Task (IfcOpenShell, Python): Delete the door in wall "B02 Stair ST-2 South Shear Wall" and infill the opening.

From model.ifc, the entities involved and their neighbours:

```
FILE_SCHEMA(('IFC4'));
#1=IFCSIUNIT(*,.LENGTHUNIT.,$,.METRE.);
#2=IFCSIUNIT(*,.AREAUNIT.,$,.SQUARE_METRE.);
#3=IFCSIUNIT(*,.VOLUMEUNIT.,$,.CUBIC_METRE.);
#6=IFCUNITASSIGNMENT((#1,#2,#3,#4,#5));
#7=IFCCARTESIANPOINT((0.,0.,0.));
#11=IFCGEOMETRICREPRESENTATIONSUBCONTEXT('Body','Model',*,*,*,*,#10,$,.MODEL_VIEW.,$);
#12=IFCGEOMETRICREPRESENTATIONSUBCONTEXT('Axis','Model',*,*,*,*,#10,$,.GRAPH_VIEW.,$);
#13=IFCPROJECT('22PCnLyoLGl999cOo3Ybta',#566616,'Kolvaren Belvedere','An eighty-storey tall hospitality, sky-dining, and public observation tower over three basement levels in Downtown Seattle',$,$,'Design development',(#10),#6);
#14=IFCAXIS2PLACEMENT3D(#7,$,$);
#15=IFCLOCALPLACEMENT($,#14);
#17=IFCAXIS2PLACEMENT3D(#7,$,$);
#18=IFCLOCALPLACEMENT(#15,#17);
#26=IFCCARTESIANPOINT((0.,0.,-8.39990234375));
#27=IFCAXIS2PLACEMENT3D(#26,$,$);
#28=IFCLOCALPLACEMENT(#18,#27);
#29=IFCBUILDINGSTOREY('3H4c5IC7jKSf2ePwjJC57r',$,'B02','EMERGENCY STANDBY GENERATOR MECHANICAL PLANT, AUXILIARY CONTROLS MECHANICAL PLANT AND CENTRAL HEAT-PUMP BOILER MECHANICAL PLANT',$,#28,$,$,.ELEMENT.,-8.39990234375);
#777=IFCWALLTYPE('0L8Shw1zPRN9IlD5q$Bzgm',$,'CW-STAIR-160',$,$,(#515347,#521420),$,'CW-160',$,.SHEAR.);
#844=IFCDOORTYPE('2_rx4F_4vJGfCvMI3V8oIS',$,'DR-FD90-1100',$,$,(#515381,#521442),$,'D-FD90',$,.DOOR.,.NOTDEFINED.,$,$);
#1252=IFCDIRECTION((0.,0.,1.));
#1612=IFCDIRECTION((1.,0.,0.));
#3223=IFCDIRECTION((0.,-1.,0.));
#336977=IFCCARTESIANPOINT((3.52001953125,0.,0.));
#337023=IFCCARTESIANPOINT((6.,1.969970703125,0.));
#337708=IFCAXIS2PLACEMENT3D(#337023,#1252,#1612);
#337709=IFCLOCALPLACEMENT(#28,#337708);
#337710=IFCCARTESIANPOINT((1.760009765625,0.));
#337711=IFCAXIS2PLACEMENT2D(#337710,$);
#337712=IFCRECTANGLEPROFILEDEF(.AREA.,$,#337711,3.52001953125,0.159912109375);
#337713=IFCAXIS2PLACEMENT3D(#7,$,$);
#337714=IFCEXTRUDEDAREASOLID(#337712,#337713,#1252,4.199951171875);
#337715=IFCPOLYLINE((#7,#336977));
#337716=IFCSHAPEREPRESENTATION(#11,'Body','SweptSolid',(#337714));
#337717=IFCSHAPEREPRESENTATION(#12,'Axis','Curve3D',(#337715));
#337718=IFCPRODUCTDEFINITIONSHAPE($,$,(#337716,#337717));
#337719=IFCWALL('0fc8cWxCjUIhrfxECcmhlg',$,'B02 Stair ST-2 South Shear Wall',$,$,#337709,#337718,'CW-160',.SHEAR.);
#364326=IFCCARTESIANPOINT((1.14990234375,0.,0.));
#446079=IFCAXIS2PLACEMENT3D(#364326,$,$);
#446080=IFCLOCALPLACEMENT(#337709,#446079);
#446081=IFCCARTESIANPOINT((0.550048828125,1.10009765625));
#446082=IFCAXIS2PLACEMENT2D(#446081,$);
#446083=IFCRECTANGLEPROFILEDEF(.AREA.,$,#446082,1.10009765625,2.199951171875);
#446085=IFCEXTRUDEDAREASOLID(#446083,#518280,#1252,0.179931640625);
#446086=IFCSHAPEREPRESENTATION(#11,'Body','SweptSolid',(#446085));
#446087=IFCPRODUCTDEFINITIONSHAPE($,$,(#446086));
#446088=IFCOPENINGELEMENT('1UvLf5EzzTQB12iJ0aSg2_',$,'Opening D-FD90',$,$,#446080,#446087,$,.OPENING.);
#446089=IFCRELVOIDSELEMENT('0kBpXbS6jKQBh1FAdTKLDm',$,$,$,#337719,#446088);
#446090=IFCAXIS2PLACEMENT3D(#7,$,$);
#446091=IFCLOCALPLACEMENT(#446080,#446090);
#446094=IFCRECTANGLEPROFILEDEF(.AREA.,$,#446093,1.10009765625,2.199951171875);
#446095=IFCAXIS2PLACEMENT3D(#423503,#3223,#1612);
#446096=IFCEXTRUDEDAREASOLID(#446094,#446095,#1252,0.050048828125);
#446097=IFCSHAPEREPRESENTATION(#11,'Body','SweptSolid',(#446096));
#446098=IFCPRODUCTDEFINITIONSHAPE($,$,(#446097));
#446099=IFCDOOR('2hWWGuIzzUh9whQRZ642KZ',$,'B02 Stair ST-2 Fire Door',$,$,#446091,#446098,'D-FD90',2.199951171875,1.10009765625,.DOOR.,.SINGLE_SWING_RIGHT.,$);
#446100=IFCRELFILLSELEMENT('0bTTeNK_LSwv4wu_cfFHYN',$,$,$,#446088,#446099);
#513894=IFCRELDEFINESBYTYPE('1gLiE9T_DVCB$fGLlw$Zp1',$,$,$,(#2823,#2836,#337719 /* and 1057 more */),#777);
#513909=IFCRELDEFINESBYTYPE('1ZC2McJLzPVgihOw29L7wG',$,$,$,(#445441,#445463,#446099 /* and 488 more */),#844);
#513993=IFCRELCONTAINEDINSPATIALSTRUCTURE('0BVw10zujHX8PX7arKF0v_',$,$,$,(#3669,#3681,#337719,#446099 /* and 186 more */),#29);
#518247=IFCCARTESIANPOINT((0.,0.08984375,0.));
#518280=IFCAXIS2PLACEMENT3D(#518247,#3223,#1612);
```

```python
import ifcopenshell
import ifcopenshell.api.feature
import ifcopenshell.api.root
import ifcopenshell.geom
import ifcopenshell.util.shape

model = ifcopenshell.open("model.ifc")
settings = ifcopenshell.geom.settings()


def volume(element):
    """Net volume in cubic metres, openings subtracted."""
    shape = ifcopenshell.geom.create_shape(settings, element)
    return ifcopenshell.util.shape.get_volume(shape.geometry)


door = model.by_guid("2hWWGuIzzUh9whQRZ642KZ")
opening = door.FillsVoids[0].RelatingOpeningElement
wall = opening.VoidsElements[0].RelatingBuildingElement
before = volume(wall)

ifcopenshell.api.root.remove_product(model, product=door)
ifcopenshell.api.feature.remove_feature(model, feature=opening)

after = volume(wall)

print(f"wall volume {before:.3f} -> {after:.3f} m3")

model.write("model_rev.ifc")
```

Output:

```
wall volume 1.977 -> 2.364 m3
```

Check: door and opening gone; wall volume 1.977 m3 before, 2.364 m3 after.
